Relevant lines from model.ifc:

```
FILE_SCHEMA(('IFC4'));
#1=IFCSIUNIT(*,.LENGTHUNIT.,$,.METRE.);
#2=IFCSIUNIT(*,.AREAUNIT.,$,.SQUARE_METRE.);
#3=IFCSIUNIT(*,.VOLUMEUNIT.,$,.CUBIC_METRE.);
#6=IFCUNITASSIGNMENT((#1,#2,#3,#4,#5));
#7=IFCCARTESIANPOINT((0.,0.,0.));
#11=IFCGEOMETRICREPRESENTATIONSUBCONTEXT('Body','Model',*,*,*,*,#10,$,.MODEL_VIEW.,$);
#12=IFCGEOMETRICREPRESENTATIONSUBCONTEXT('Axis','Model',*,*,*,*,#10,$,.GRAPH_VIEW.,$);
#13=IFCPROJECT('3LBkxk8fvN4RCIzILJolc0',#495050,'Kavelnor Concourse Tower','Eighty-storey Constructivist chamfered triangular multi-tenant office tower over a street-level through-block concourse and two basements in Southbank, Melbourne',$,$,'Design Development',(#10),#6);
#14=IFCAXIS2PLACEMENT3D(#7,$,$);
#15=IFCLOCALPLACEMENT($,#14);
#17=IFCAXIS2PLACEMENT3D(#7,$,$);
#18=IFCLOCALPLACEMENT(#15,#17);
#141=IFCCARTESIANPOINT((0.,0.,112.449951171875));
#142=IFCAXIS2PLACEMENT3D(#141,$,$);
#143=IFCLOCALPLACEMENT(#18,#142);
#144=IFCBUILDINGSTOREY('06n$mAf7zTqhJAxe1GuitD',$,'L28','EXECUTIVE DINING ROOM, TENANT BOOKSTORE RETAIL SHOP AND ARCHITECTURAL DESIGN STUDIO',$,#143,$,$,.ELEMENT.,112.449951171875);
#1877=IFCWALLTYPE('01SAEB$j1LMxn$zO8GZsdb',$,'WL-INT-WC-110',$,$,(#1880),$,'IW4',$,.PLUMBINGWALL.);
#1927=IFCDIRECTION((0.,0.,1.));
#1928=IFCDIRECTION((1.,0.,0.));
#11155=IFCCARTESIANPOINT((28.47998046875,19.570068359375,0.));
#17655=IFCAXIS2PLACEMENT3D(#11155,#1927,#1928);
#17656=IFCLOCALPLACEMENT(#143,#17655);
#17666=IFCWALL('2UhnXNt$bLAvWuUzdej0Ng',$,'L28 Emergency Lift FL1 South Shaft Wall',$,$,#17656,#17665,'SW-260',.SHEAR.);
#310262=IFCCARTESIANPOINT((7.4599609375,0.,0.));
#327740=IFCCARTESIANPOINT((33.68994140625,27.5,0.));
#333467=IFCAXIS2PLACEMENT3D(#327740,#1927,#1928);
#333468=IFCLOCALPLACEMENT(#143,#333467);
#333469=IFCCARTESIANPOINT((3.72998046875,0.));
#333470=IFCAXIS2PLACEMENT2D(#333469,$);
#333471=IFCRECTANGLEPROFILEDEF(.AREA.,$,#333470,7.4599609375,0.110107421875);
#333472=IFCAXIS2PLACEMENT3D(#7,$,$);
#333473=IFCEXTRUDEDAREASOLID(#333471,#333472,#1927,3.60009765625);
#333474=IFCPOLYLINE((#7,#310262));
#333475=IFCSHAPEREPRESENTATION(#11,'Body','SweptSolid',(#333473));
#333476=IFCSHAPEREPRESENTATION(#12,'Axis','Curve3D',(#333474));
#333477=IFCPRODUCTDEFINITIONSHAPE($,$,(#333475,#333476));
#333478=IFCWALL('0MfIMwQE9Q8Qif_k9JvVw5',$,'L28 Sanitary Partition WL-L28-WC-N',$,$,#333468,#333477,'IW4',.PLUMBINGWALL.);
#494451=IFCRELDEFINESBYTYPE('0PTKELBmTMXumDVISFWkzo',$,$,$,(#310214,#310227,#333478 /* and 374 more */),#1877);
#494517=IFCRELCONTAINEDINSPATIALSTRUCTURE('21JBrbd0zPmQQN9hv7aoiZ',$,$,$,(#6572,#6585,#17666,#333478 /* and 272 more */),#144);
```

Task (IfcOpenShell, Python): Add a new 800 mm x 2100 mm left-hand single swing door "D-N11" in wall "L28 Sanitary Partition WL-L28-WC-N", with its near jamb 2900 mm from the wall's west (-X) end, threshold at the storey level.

```python
import numpy as np
import ifcopenshell
import ifcopenshell.api.feature
import ifcopenshell.api.geometry
import ifcopenshell.api.root
import ifcopenshell.api.spatial
import ifcopenshell.geom
import ifcopenshell.util.element
import ifcopenshell.util.placement
import ifcopenshell.util.representation
import ifcopenshell.util.shape
import ifcopenshell.util.unit

model = ifcopenshell.open("model.ifc")
unit_scale = ifcopenshell.util.unit.calculate_unit_scale(model)
settings = ifcopenshell.geom.settings()


def volume(element):
    """Net volume in cubic metres, openings subtracted."""
    shape = ifcopenshell.geom.create_shape(settings, element)
    return ifcopenshell.util.shape.get_volume(shape.geometry)


wall = model.by_guid("0MfIMwQE9Q8Qif_k9JvVw5")
storey = ifcopenshell.util.element.get_container(wall, ifc_class="IfcBuildingStorey")
context = ifcopenshell.util.representation.get_context(model, "Model", "Body", "MODEL_VIEW")
before = volume(wall)

width, height, from_end, sill = 0.8, 2.1, 2.9, 0.0  # metres

# The wall runs along its own X axis, and the end named is its -X end.
wall_shape = ifcopenshell.geom.create_shape(settings, wall)
x, y, z = ifcopenshell.util.shape.get_vertices(wall_shape.geometry).T
start = x.min() + from_end
face, thickness = float(y.min()), float(y.max() - y.min())
wall_matrix = ifcopenshell.util.placement.get_local_placement(wall.ObjectPlacement)
level = ifcopenshell.util.placement.get_local_placement(storey.ObjectPlacement)[2, 3]


def in_wall(x, y):
    """Placement at x, y metres in the wall's axes, at sill height."""
    matrix = wall_matrix.copy()
    matrix[:, 3] = wall_matrix @ np.array([x / unit_scale, y / unit_scale, 0.0, 1.0])
    matrix[2, 3] = level + sill / unit_scale
    return matrix


# Opening: a box that overshoots both wall faces by 50 mm.
opening = ifcopenshell.api.root.create_entity(model, ifc_class="IfcOpeningElement", predefined_type="OPENING")
box = ifcopenshell.api.geometry.add_wall_representation(
    model, context=context, length=width, height=height, thickness=thickness + 0.1
)
ifcopenshell.api.geometry.assign_representation(model, product=opening, representation=box)
ifcopenshell.api.geometry.edit_object_placement(model, product=opening, matrix=in_wall(start, face - 0.05), is_si=False)
ifcopenshell.api.feature.add_feature(model, feature=opening, element=wall)

door = ifcopenshell.api.root.create_entity(model, ifc_class="IfcDoor", name="D-N11", predefined_type="DOOR")
door.OverallWidth, door.OverallHeight = width / unit_scale, height / unit_scale
door.OperationType = "SINGLE_SWING_LEFT"
body = ifcopenshell.api.geometry.add_door_representation(
    model,
    context=context,
    overall_width=door.OverallWidth,
    overall_height=door.OverallHeight,
    operation_type="SINGLE_SWING_LEFT",
    lining_properties={"LiningDepth": thickness / unit_scale, "ThresholdDepth": thickness / unit_scale},
)
ifcopenshell.api.geometry.assign_representation(model, product=door, representation=body)
ifcopenshell.api.spatial.assign_container(model, products=[door], relating_structure=storey)
ifcopenshell.api.feature.add_filling(model, opening=opening, element=door)

# The lining spans the wall, so the door starts at the wall face.
ifcopenshell.api.geometry.edit_object_placement(model, product=door, matrix=in_wall(start, face), is_si=False)

after = volume(wall)

print(f"wall volume {before:.3f} -> {after:.3f} m3")

model.write("model_rev.ifc")
```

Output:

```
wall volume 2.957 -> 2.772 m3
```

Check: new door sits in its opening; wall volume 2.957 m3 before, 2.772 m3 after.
